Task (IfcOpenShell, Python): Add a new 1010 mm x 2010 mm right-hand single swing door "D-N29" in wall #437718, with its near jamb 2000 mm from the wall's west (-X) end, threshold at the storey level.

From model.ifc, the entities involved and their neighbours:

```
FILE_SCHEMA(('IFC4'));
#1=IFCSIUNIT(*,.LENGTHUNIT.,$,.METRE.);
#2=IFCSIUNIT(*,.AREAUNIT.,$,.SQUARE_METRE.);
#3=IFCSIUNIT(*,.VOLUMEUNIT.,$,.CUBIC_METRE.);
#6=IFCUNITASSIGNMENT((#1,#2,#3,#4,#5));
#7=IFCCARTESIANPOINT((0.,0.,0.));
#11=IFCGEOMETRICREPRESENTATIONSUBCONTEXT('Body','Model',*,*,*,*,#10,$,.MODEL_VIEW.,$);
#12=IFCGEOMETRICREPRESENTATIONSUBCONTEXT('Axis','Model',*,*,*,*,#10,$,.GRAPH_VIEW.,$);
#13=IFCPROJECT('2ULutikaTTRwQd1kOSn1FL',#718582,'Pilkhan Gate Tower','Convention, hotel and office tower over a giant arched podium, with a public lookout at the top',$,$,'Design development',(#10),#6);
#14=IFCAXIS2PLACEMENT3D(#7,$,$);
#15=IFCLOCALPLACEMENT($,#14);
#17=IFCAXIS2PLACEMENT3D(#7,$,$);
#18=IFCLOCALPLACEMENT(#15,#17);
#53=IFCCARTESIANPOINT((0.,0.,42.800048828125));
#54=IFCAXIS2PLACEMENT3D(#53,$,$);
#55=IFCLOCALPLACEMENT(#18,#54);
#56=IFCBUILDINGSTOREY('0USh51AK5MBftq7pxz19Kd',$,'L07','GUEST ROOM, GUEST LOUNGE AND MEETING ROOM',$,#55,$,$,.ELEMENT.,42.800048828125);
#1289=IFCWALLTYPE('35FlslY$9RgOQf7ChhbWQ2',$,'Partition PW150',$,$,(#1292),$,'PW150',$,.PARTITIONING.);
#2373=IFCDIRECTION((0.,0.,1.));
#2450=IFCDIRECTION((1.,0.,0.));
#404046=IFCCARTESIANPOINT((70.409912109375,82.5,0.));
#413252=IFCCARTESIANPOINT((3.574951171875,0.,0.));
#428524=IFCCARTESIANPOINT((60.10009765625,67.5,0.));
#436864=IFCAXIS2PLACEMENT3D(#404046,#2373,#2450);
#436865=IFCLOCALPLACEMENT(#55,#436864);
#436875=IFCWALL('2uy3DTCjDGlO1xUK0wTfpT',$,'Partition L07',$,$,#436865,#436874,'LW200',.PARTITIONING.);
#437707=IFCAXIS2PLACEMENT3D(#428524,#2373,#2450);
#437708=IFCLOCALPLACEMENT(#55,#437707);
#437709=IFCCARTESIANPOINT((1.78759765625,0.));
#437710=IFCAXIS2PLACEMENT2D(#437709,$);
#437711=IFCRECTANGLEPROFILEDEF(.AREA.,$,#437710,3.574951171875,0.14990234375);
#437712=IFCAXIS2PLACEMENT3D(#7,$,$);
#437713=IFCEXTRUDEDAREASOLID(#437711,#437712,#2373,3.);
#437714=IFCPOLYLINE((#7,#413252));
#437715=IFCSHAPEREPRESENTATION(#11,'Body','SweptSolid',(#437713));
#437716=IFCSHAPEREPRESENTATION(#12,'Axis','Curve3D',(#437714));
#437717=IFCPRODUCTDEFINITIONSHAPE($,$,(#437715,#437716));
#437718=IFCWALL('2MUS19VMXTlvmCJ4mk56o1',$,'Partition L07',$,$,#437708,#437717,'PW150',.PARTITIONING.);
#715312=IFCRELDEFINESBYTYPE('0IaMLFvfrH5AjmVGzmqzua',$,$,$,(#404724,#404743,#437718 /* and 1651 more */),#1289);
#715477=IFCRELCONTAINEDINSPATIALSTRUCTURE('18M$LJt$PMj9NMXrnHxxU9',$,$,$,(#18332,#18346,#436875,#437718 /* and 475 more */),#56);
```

```python
import numpy as np
import ifcopenshell
import ifcopenshell.api.feature
import ifcopenshell.api.geometry
import ifcopenshell.api.root
import ifcopenshell.api.spatial
import ifcopenshell.geom
import ifcopenshell.util.element
import ifcopenshell.util.placement
import ifcopenshell.util.representation
import ifcopenshell.util.shape
import ifcopenshell.util.unit

model = ifcopenshell.open("model.ifc")
unit_scale = ifcopenshell.util.unit.calculate_unit_scale(model)
settings = ifcopenshell.geom.settings()


def volume(element):
    """Net volume in cubic metres, openings subtracted."""
    shape = ifcopenshell.geom.create_shape(settings, element)
    return ifcopenshell.util.shape.get_volume(shape.geometry)


wall = model.by_guid("2MUS19VMXTlvmCJ4mk56o1")
storey = ifcopenshell.util.element.get_container(wall, ifc_class="IfcBuildingStorey")
context = ifcopenshell.util.representation.get_context(model, "Model", "Body", "MODEL_VIEW")
before = volume(wall)

width, height, from_end, sill = 1.01, 2.01, 2, 0.0  # metres

# The wall runs along its own X axis, and the end named is its -X end.
wall_shape = ifcopenshell.geom.create_shape(settings, wall)
x, y, z = ifcopenshell.util.shape.get_vertices(wall_shape.geometry).T
start = x.min() + from_end
face, thickness = float(y.min()), float(y.max() - y.min())
wall_matrix = ifcopenshell.util.placement.get_local_placement(wall.ObjectPlacement)
level = ifcopenshell.util.placement.get_local_placement(storey.ObjectPlacement)[2, 3]


def in_wall(x, y):
    """Placement at x, y metres in the wall's axes, at sill height."""
    matrix = wall_matrix.copy()
    matrix[:, 3] = wall_matrix @ np.array([x / unit_scale, y / unit_scale, 0.0, 1.0])
    matrix[2, 3] = level + sill / unit_scale
    return matrix


# Opening: a box that overshoots both wall faces by 50 mm.
opening = ifcopenshell.api.root.create_entity(model, ifc_class="IfcOpeningElement", predefined_type="OPENING")
box = ifcopenshell.api.geometry.add_wall_representation(
    model, context=context, length=width, height=height, thickness=thickness + 0.1
)
ifcopenshell.api.geometry.assign_representation(model, product=opening, representation=box)
ifcopenshell.api.geometry.edit_object_placement(model, product=opening, matrix=in_wall(start, face - 0.05), is_si=False)
ifcopenshell.api.feature.add_feature(model, feature=opening, element=wall)

door = ifcopenshell.api.root.create_entity(model, ifc_class="IfcDoor", name="D-N29", predefined_type="DOOR")
door.OverallWidth, door.OverallHeight = width / unit_scale, height / unit_scale
door.OperationType = "SINGLE_SWING_RIGHT"
body = ifcopenshell.api.geometry.add_door_representation(
    model,
    context=context,
    overall_width=door.OverallWidth,
    overall_height=door.OverallHeight,
    operation_type="SINGLE_SWING_RIGHT",
    lining_properties={"LiningDepth": thickness / unit_scale, "ThresholdDepth": thickness / unit_scale},
)
ifcopenshell.api.geometry.assign_representation(model, product=door, representation=body)
ifcopenshell.api.spatial.assign_container(model, products=[door], relating_structure=storey)
ifcopenshell.api.feature.add_filling(model, opening=opening, element=door)

# The lining spans the wall, so the door starts at the wall face.
ifcopenshell.api.geometry.edit_object_placement(model, product=door, matrix=in_wall(start, face), is_si=False)

after = volume(wall)

print(f"wall volume {before:.3f} -> {after:.3f} m3")

model.write("model_rev.ifc")
```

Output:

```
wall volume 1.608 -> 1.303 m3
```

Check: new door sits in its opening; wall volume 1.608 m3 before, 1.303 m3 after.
